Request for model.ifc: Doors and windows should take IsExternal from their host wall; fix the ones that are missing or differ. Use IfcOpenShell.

First a look at what the model holds.

```python
import ifcopenshell
import ifcopenshell.util.element

model = ifcopenshell.open("model.ifc")
print(model.schema)
seen = {}
for e in model.by_type("IfcDoor") + model.by_type("IfcWindow"):
    if not e.FillsVoids:
        continue
    host = e.FillsVoids[0].RelatingOpeningElement.VoidsElements[0].RelatingBuildingElement
    own = ifcopenshell.util.element.get_pset(e, f"Pset_{e.is_a()[3:].removesuffix('StandardCase')}Common", "IsExternal")
    wall = ifcopenshell.util.element.get_pset(host, "Pset_WallCommon", "IsExternal")
    seen[e.is_a(), own, wall] = seen.get((e.is_a(), own, wall), 0) + 1
for (cls, own, wall), count in sorted(seen.items(), key=str):
    print(count, cls, "IsExternal:", own, "| host wall:", wall)
```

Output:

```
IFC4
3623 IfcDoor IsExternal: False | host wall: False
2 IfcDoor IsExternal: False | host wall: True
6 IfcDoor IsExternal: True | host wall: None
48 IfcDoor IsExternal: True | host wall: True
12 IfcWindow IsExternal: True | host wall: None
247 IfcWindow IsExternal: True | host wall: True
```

```python
import ifcopenshell
import ifcopenshell.api.pset
import ifcopenshell.util.element

model = ifcopenshell.open("model.ifc")

count = 0
for ifc_class, pset_name in (("IfcDoor", "Pset_DoorCommon"), ("IfcWindow", "Pset_WindowCommon")):
    for e in model.by_type(ifc_class):
        if not e.FillsVoids:
            continue
        host = e.FillsVoids[0].RelatingOpeningElement.VoidsElements[0].RelatingBuildingElement
        external = ifcopenshell.util.element.get_pset(host, "Pset_WallCommon", "IsExternal")
        if external is None or ifcopenshell.util.element.get_pset(e, pset_name, "IsExternal") == external:
            continue
        pset = ifcopenshell.api.pset.add_pset(model, product=e, name=pset_name)
        ifcopenshell.api.pset.edit_pset(model, pset=pset, properties={"IsExternal": external})
        count += 1

print(count, "updated")

model.write("model_v2.ifc")
```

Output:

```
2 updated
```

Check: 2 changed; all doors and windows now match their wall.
